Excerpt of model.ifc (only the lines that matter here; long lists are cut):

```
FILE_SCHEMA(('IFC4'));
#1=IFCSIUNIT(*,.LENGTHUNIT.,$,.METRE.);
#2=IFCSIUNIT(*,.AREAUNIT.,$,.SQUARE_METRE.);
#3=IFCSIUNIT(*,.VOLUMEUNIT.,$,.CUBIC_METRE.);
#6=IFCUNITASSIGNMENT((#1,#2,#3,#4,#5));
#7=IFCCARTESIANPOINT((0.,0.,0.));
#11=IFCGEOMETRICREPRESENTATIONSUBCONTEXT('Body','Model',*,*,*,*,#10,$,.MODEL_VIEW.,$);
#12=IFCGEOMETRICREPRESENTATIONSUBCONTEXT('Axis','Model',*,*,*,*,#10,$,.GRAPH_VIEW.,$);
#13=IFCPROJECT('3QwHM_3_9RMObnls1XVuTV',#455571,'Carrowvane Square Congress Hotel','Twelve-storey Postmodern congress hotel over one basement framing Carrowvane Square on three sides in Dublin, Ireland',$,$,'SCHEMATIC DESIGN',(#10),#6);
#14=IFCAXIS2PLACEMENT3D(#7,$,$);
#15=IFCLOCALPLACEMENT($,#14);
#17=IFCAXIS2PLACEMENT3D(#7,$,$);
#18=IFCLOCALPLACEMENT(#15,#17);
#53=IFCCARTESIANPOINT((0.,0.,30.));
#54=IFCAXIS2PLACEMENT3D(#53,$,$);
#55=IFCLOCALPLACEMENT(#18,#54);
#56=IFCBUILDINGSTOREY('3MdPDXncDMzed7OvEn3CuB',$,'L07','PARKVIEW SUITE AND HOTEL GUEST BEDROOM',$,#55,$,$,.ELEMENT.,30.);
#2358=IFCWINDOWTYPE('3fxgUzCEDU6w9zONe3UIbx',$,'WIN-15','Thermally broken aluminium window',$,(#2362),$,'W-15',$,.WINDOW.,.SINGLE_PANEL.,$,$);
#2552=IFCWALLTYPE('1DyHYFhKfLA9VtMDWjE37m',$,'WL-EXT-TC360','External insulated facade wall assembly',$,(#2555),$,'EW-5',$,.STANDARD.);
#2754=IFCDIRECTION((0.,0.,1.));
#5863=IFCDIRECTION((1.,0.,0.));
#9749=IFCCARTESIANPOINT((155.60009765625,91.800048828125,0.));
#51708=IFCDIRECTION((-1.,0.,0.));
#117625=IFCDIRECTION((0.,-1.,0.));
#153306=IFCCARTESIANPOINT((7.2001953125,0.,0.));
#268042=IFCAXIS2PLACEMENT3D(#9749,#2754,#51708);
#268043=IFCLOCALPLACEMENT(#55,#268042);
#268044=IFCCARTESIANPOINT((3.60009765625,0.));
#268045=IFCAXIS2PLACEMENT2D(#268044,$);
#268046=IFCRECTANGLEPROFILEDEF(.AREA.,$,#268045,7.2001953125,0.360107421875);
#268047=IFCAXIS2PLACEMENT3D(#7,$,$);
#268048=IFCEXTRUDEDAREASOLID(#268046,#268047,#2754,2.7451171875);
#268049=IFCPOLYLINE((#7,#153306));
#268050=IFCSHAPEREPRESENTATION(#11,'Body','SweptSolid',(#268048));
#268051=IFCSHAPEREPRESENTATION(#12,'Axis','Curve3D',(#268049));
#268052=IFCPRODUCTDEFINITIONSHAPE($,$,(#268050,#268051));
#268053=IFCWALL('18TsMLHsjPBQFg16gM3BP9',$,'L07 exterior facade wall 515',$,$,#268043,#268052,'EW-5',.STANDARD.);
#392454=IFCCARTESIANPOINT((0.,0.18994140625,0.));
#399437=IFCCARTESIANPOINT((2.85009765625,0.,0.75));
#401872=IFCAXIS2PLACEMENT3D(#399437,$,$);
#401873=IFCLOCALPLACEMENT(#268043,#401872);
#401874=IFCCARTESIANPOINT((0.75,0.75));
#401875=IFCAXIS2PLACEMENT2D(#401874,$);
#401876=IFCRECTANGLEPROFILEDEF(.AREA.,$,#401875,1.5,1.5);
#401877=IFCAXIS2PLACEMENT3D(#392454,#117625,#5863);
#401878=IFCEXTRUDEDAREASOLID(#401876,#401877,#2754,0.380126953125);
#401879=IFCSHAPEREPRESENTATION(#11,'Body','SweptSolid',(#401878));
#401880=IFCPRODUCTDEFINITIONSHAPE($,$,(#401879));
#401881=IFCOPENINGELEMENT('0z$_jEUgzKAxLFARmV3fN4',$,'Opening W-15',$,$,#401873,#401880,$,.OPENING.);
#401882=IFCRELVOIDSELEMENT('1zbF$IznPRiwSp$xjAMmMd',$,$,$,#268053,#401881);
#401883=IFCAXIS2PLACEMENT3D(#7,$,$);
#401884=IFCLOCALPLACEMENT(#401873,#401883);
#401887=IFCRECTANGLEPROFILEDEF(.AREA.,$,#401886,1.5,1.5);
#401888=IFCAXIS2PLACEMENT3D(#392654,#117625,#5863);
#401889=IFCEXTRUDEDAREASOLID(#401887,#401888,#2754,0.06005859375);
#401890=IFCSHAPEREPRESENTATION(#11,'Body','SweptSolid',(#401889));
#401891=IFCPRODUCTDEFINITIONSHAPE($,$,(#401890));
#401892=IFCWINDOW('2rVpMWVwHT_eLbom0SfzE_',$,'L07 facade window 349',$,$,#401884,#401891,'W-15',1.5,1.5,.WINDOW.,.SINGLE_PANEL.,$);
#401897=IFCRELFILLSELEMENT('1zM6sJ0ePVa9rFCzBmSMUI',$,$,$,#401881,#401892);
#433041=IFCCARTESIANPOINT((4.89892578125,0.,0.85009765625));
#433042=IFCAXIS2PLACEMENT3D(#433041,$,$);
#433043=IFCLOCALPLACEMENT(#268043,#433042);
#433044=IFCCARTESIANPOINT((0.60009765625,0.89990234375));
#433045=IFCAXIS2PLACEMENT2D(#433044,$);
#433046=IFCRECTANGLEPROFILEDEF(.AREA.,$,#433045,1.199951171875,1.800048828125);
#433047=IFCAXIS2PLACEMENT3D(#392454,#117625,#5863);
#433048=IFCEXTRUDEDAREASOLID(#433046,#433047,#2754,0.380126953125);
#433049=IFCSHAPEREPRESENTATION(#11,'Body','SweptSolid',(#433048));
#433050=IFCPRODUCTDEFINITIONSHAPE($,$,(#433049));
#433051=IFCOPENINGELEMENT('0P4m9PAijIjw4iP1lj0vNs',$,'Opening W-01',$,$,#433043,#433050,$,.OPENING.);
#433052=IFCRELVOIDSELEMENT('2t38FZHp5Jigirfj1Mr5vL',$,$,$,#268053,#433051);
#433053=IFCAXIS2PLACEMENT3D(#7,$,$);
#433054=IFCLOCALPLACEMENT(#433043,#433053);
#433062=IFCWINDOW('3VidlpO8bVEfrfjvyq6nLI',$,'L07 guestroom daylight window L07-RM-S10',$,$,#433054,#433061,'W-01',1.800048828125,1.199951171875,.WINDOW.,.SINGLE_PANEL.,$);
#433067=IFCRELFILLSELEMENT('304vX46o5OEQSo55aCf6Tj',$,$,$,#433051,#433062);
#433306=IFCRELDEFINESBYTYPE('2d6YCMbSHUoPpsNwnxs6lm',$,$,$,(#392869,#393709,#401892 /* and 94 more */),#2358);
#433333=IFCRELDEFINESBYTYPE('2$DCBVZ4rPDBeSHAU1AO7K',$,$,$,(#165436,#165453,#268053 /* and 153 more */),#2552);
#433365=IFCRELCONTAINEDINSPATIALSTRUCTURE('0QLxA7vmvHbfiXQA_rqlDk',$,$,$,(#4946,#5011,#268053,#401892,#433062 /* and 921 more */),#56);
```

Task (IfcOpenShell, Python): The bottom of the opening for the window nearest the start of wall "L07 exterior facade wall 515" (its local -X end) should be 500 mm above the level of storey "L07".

```python
import numpy as np
import ifcopenshell
import ifcopenshell.api.geometry
import ifcopenshell.geom
import ifcopenshell.util.element
import ifcopenshell.util.placement
import ifcopenshell.util.shape
import ifcopenshell.util.unit

model = ifcopenshell.open("model.ifc")
unit_scale = ifcopenshell.util.unit.calculate_unit_scale(model)

window = model.by_guid("2rVpMWVwHT_eLbom0SfzE_")
opening = window.FillsVoids[0].RelatingOpeningElement
storey = ifcopenshell.util.element.get_container(window, ifc_class="IfcBuildingStorey")
level = ifcopenshell.util.placement.get_local_placement(storey.ObjectPlacement)[2, 3]

# The opening's origin need not be at the sill, so measure its lowest point.
shape = ifcopenshell.geom.create_shape(ifcopenshell.geom.settings(), opening)
bottom = ifcopenshell.util.shape.get_shape_bottom_elevation(shape, shape.geometry) / unit_scale
dz = level + 0.5 / unit_scale - bottom

shift = np.array([0.0, 0.0, dz])
# The window is placed relative to its opening, so it follows when the opening moves.
matrix = ifcopenshell.util.placement.get_local_placement(opening.ObjectPlacement)
matrix[:3, 3] += shift
ifcopenshell.api.geometry.edit_object_placement(
    model, product=opening, matrix=matrix, is_si=False, should_transform_children=True
)

print(f"moved by {dz * unit_scale:+.3f} m")

model.write("model-out.ifc")
```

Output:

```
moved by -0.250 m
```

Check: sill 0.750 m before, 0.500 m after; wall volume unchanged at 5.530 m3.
